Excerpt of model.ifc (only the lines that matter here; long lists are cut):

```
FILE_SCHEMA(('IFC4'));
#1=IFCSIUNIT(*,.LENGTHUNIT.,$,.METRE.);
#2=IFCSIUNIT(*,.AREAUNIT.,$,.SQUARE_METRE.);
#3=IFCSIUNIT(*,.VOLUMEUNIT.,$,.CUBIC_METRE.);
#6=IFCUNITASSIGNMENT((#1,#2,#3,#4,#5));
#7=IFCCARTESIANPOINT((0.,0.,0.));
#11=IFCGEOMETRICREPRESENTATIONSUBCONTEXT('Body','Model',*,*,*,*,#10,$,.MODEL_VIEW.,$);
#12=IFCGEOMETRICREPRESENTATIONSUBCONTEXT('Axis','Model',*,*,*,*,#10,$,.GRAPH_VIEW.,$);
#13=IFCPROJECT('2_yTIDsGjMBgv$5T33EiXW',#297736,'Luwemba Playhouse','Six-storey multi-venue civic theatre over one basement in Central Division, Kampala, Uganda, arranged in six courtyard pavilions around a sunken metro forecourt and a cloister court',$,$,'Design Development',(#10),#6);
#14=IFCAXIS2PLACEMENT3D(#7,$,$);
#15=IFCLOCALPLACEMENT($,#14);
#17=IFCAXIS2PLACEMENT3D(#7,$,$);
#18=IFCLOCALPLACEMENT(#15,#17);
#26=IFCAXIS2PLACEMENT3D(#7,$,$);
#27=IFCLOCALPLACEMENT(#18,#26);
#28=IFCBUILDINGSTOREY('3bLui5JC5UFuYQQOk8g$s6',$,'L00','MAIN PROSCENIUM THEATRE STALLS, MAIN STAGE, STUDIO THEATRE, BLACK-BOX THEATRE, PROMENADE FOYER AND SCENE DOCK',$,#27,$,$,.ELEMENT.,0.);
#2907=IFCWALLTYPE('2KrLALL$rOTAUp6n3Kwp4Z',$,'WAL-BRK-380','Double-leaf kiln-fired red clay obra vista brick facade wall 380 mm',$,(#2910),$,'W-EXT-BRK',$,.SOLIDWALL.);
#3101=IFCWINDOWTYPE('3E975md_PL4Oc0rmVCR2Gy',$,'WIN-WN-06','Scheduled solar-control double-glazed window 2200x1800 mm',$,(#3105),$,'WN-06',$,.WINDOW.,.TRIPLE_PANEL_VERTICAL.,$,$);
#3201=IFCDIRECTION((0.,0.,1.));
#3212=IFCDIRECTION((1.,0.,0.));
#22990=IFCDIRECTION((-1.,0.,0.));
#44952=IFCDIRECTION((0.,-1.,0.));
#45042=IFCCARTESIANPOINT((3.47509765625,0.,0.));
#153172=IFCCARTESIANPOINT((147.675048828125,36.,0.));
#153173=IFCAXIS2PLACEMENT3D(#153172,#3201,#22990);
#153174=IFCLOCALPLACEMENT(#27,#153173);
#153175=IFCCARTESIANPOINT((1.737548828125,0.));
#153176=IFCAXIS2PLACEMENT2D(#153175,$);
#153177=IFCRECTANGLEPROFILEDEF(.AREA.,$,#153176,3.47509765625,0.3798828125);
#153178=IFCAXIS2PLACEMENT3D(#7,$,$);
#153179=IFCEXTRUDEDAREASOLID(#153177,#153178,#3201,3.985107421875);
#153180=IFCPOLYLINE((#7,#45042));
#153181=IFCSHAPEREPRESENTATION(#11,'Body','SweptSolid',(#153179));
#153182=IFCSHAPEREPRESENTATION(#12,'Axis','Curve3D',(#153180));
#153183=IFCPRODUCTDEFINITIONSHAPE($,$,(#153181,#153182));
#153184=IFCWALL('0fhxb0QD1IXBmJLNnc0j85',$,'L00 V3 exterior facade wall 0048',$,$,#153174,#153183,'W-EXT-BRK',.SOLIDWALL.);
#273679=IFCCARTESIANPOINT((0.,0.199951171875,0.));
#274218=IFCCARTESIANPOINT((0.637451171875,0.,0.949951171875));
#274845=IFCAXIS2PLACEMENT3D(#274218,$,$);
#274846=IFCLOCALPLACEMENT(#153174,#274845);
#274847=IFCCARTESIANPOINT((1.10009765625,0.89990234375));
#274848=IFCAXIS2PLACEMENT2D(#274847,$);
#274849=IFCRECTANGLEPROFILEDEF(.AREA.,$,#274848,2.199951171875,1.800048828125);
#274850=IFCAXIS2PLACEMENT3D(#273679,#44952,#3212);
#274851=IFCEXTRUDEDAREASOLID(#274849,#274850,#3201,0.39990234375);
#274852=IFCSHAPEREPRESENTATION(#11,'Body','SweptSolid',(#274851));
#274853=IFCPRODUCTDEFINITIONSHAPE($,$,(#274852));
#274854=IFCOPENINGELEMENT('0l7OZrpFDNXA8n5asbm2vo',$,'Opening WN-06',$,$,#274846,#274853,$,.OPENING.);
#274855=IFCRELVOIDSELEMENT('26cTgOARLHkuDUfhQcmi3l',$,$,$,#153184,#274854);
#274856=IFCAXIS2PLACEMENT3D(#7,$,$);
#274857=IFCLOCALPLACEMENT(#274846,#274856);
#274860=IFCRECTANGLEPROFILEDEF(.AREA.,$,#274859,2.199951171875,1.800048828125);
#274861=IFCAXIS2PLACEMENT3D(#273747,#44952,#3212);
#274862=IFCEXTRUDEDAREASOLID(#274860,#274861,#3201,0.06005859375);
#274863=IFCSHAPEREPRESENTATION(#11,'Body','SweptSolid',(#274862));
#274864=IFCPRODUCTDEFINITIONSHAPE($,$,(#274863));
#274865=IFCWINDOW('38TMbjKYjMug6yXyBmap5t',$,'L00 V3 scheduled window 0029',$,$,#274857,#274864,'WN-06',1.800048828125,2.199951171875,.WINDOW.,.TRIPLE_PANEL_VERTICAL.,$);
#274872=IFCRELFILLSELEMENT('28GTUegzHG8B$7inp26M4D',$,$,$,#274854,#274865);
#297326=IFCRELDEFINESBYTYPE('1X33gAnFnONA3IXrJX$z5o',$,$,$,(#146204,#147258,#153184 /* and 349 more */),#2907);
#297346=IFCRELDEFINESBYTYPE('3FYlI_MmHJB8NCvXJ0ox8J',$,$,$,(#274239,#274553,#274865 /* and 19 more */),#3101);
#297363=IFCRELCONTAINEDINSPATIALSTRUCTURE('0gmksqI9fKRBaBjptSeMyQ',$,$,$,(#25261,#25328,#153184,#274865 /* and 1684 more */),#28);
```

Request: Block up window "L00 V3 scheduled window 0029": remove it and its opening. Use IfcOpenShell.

```python
import ifcopenshell
import ifcopenshell.api.feature
import ifcopenshell.api.root
import ifcopenshell.geom
import ifcopenshell.util.shape

model = ifcopenshell.open("model.ifc")
settings = ifcopenshell.geom.settings()


def volume(element):
    """Net volume in cubic metres, openings subtracted."""
    shape = ifcopenshell.geom.create_shape(settings, element)
    return ifcopenshell.util.shape.get_volume(shape.geometry)


window = model.by_guid("38TMbjKYjMug6yXyBmap5t")
opening = window.FillsVoids[0].RelatingOpeningElement
wall = opening.VoidsElements[0].RelatingBuildingElement
before = volume(wall)

ifcopenshell.api.root.remove_product(model, product=window)
ifcopenshell.api.feature.remove_feature(model, feature=opening)

after = volume(wall)

print(f"wall volume {before:.3f} -> {after:.3f} m3")

model.write("model-out.ifc")
```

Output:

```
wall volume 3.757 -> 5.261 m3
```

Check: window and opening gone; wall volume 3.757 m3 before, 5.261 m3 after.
